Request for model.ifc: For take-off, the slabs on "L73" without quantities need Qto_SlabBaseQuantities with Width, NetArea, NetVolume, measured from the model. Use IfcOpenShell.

First a look at what the model holds.

```python
import ifcopenshell
import ifcopenshell.util.element
import ifcopenshell.util.unit

model = ifcopenshell.open("model.ifc")
print(model.schema)
for unit_type in ("LENGTHUNIT", "AREAUNIT", "VOLUMEUNIT"):
    print(unit_type, ifcopenshell.util.unit.calculate_unit_scale(model, unit_type))
storey = next(s for s in model.by_type("IfcBuildingStorey") if s.Name == "L73")
slabs = [e for e in ifcopenshell.util.element.get_decomposition(storey) if e.is_a("IfcSlab")]
for e in sorted(slabs, key=lambda e: e.id()):
    print(e.id(), e.is_a(), e.Name, list(ifcopenshell.util.element.get_psets(e, qtos_only=True)), sep=" | ")
```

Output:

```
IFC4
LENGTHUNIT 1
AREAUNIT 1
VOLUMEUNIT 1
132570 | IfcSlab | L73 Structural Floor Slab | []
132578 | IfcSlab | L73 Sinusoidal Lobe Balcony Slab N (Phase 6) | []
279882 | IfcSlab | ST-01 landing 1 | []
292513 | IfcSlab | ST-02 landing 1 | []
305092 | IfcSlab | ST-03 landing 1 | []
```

```python
import ifcopenshell
import ifcopenshell.api.pset
import ifcopenshell.geom
import ifcopenshell.util.element
import ifcopenshell.util.shape
import ifcopenshell.util.unit

model = ifcopenshell.open("model.ifc")
unit_scale = ifcopenshell.util.unit.calculate_unit_scale(model)
area_scale = ifcopenshell.util.unit.calculate_unit_scale(model, "AREAUNIT")
volume_scale = ifcopenshell.util.unit.calculate_unit_scale(model, "VOLUMEUNIT")
settings = ifcopenshell.geom.settings()

storey = next(s for s in model.by_type("IfcBuildingStorey") if s.Name == "L73")
slabs = [e for e in ifcopenshell.util.element.get_decomposition(storey) if e.is_a("IfcSlab")]

for e in sorted(slabs, key=lambda e: e.id()):
    if ifcopenshell.util.element.get_psets(e, qtos_only=True, should_inherit=False):
        continue
    # Geometry comes back in metres, in the element's own axes.
    shape = ifcopenshell.geom.create_shape(settings, e)
    values = {
        "Width": ifcopenshell.util.shape.get_z(shape.geometry) / unit_scale,
        "NetArea": ifcopenshell.util.shape.get_footprint_area(shape.geometry) / area_scale,
        "NetVolume": ifcopenshell.util.shape.get_volume(shape.geometry) / volume_scale,
    }
    qto = ifcopenshell.api.pset.add_qto(model, product=e, name="Qto_SlabBaseQuantities")
    ifcopenshell.api.pset.edit_qto(model, qto=qto, properties=values)
    print(e.id(), {k: round(v, 3) for k, v in values.items()})

model.write("model_updated.ifc")
```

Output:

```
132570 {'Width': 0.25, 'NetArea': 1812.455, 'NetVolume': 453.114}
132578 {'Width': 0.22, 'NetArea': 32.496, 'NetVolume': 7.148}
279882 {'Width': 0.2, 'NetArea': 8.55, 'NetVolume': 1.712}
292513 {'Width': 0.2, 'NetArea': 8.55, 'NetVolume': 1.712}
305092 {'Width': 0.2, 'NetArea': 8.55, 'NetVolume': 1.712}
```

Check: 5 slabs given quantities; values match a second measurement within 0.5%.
